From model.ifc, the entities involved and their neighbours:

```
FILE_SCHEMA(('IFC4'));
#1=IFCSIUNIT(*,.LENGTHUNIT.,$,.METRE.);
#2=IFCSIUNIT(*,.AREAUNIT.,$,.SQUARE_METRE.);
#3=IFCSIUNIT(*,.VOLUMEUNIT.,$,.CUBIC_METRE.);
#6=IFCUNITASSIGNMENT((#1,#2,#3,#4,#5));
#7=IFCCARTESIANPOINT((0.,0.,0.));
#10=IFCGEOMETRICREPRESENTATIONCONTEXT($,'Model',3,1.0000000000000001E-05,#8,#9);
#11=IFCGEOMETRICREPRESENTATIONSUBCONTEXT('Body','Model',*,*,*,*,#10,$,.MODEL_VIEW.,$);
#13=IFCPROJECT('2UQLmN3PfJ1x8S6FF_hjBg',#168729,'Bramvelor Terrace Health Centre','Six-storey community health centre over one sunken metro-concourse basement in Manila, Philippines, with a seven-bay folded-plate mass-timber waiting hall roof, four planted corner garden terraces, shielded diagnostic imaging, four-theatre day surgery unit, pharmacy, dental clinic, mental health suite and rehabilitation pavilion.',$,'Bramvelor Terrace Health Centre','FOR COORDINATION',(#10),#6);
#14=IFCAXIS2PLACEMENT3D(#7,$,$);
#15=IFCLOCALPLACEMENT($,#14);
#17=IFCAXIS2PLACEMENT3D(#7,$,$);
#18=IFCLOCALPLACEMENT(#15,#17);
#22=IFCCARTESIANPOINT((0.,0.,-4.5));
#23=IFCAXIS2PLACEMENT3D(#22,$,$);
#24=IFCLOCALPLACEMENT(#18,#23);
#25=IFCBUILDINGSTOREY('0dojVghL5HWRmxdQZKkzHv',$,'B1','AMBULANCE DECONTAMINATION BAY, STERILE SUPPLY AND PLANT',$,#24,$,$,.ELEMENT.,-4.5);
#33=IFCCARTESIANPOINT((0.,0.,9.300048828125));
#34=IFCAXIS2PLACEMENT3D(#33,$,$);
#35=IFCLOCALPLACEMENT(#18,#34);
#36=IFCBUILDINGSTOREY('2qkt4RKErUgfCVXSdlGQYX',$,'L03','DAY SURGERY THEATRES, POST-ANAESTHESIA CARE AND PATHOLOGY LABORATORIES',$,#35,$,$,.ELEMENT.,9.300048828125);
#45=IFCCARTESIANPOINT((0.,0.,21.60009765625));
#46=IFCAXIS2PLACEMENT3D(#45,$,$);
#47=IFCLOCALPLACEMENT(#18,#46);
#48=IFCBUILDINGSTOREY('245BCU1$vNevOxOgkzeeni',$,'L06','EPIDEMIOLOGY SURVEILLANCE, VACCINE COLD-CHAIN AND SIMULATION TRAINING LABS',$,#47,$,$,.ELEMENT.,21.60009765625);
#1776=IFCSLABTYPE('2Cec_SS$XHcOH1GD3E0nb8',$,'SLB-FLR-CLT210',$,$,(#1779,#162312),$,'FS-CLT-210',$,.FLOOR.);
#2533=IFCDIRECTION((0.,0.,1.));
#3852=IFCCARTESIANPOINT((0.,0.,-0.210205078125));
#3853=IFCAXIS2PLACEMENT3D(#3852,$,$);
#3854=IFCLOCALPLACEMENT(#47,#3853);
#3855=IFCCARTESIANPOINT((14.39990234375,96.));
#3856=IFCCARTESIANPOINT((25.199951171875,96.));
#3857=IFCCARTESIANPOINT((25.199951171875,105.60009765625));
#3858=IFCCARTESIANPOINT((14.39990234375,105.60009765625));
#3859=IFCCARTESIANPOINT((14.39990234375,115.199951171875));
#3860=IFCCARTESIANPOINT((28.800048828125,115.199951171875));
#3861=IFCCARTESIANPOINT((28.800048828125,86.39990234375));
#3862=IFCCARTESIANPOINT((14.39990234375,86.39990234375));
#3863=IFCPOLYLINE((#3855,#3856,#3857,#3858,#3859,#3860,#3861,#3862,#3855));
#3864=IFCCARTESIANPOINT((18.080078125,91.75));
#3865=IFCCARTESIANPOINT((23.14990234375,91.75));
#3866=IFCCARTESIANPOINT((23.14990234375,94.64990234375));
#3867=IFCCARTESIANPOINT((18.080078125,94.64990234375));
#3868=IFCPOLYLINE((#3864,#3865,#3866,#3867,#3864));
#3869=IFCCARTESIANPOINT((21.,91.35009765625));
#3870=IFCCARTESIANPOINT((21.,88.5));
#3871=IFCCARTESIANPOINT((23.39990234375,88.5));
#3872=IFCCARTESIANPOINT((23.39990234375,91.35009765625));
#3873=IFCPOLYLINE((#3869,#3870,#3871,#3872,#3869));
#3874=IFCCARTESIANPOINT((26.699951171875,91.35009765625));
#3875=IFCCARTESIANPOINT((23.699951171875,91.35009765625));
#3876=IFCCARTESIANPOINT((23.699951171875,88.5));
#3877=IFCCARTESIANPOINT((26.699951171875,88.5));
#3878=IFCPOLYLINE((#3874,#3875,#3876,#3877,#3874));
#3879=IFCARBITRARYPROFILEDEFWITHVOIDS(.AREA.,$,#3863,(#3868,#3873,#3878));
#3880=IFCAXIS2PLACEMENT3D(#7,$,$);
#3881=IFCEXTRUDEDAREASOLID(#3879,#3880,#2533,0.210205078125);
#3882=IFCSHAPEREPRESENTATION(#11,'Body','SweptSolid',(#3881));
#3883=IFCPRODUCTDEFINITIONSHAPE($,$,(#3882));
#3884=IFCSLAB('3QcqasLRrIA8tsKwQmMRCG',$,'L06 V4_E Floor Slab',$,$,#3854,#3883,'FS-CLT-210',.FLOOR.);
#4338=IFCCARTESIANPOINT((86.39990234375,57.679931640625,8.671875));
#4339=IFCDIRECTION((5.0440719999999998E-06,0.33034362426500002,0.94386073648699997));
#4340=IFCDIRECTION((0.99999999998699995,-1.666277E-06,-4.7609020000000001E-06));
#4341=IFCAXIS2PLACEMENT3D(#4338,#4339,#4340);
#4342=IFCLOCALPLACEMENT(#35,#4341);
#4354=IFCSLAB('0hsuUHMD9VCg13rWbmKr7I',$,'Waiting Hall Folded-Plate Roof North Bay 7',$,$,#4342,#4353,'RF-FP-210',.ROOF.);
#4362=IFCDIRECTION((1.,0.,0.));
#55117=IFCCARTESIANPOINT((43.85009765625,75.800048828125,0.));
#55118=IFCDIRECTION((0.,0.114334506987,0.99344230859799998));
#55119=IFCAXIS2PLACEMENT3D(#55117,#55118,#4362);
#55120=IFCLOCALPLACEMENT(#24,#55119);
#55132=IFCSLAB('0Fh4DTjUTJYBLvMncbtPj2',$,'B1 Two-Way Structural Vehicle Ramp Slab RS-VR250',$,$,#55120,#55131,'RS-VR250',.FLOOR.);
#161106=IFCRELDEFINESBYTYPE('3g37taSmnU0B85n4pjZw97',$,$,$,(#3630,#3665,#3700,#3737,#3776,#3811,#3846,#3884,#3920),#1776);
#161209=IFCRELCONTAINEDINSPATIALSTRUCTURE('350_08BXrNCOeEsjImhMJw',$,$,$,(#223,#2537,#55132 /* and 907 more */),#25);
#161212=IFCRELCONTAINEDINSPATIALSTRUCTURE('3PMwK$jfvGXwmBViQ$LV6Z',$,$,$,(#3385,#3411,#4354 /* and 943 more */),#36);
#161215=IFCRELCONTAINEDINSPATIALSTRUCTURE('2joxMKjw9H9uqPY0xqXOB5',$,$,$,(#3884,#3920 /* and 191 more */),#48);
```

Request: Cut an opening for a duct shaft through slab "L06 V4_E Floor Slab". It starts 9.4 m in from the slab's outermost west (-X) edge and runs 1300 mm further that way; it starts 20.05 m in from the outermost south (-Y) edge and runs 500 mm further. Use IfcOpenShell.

```python
import numpy as np
import ifcopenshell
import ifcopenshell.api.feature
import ifcopenshell.api.geometry
import ifcopenshell.api.root
import ifcopenshell.geom
import ifcopenshell.util.placement
import ifcopenshell.util.representation
import ifcopenshell.util.shape
import ifcopenshell.util.unit

model = ifcopenshell.open("model.ifc")
unit_scale = ifcopenshell.util.unit.calculate_unit_scale(model)
settings = ifcopenshell.geom.settings()


def volume(element):
    """Net volume in cubic metres, openings subtracted."""
    shape = ifcopenshell.geom.create_shape(settings, element)
    return ifcopenshell.util.shape.get_volume(shape.geometry)


slab = model.by_guid("3QcqasLRrIA8tsKwQmMRCG")
before = volume(slab)

# Extent in the slab's own axes, in metres. The edges named are its -X and -Y sides.
slab_shape = ifcopenshell.geom.create_shape(settings, slab)
vertices = ifcopenshell.util.shape.get_vertices(slab_shape.geometry)
x_min, y_min, bottom = vertices.min(axis=0)
top = vertices[:, 2].max()

opening = ifcopenshell.api.root.create_entity(model, ifc_class="IfcOpeningElement", name="Duct shaft opening", predefined_type="OPENING")
context = ifcopenshell.util.representation.get_context(model, "Model", "Body", "MODEL_VIEW")
width, depth = 1.3, 0.5
outline = [(0.0, 0.0), (width, 0.0), (width, depth), (0.0, depth), (0.0, 0.0)]
# Overshoot both faces by 50 mm so the cut is clean.
shape = ifcopenshell.api.geometry.add_slab_representation(
    model, context=context, depth=top - bottom + 0.1, polyline=outline
)
ifcopenshell.api.geometry.assign_representation(model, product=opening, representation=shape)

matrix = ifcopenshell.util.placement.get_local_placement(slab.ObjectPlacement)
matrix[:, 3] = matrix @ np.append(np.array([x_min + 9.4, y_min + 20.05, bottom - 0.05]) / unit_scale, 1.0)
ifcopenshell.api.geometry.edit_object_placement(model, product=opening, matrix=matrix, is_si=False)
ifcopenshell.api.feature.add_feature(model, feature=opening, element=slab)

after = volume(slab)

print(f"slab volume {before:.3f} -> {after:.3f} m3")

model.write("model-out.ifc")
```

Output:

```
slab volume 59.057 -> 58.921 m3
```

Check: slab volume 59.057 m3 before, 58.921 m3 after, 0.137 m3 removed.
